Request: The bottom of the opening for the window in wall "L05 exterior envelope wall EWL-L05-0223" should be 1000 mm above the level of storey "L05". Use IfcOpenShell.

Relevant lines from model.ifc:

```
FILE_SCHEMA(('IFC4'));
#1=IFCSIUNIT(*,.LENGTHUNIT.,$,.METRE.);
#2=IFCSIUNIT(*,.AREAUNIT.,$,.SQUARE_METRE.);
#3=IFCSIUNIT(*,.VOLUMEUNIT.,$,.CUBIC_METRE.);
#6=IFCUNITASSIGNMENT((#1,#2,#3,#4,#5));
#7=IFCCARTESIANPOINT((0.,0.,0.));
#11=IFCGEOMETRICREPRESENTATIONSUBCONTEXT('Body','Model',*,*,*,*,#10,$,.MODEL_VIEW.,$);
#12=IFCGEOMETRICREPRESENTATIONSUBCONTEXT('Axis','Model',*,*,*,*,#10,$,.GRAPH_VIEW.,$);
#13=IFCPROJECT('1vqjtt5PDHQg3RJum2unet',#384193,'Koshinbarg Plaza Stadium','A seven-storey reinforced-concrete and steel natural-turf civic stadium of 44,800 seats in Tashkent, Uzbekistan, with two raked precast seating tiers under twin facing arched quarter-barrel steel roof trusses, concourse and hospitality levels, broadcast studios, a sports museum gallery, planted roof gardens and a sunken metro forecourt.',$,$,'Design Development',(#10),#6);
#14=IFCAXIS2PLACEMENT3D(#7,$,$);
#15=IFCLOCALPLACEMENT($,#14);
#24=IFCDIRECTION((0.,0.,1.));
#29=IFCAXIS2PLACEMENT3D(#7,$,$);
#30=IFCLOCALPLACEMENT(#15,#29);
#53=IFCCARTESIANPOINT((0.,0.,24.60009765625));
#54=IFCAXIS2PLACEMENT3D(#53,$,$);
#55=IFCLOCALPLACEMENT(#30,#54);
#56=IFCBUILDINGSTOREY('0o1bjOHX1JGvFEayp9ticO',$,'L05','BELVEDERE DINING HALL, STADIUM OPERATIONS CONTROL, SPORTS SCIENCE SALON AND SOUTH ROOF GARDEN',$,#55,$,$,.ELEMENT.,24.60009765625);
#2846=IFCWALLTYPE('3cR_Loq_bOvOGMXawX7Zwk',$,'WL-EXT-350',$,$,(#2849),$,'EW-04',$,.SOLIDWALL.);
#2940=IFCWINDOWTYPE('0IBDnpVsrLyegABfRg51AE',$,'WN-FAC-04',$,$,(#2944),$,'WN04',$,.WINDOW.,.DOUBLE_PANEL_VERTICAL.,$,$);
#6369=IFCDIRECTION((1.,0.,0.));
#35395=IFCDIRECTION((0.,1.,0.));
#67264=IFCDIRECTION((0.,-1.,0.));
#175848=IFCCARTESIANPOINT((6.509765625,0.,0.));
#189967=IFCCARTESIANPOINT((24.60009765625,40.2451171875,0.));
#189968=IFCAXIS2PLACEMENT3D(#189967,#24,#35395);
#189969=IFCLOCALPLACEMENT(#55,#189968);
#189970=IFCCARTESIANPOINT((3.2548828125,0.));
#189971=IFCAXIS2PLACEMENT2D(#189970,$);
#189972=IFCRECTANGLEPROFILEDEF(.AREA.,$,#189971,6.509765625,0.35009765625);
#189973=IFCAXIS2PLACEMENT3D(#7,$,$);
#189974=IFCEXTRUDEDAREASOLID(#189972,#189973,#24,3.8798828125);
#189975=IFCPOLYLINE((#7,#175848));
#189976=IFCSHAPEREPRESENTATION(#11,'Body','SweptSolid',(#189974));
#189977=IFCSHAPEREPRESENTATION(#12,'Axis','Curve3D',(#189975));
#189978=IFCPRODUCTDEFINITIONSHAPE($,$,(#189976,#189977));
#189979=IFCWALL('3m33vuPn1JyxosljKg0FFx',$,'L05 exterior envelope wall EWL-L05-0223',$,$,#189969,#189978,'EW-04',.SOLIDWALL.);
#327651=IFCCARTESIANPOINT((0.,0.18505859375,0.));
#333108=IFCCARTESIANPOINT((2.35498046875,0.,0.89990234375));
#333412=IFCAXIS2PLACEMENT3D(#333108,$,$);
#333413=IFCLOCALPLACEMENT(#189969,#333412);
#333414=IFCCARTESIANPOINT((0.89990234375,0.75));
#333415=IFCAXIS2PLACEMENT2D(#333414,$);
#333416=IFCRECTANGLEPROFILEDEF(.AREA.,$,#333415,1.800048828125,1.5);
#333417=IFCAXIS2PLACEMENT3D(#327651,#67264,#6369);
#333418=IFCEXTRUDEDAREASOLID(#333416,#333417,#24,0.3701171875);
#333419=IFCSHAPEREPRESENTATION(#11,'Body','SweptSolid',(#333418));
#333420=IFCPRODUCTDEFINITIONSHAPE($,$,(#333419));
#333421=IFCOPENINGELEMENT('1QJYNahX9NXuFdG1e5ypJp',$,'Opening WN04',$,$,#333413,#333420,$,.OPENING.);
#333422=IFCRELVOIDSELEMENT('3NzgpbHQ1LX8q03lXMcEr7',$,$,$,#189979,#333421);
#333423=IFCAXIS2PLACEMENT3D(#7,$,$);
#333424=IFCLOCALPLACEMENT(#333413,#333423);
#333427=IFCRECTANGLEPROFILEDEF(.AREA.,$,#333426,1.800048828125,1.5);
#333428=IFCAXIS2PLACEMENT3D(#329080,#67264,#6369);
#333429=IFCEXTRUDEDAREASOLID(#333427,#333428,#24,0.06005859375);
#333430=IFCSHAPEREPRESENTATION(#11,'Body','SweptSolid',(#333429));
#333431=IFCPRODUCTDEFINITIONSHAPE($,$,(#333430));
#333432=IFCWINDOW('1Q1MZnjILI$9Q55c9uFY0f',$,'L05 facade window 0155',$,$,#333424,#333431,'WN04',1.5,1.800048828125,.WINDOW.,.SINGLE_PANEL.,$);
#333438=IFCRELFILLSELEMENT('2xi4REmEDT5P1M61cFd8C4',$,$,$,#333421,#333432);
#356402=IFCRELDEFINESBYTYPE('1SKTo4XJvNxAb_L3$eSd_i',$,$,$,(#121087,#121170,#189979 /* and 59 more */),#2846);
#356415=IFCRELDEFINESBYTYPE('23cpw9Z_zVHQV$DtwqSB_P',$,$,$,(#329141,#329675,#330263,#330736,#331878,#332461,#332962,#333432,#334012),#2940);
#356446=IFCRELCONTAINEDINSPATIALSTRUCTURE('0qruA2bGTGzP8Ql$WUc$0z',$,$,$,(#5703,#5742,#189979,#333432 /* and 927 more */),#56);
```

```python
import numpy as np
import ifcopenshell
import ifcopenshell.api.geometry
import ifcopenshell.geom
import ifcopenshell.util.element
import ifcopenshell.util.placement
import ifcopenshell.util.shape
import ifcopenshell.util.unit

model = ifcopenshell.open("model.ifc")
unit_scale = ifcopenshell.util.unit.calculate_unit_scale(model)

window = model.by_guid("1Q1MZnjILI$9Q55c9uFY0f")
opening = window.FillsVoids[0].RelatingOpeningElement
storey = ifcopenshell.util.element.get_container(window, ifc_class="IfcBuildingStorey")
level = ifcopenshell.util.placement.get_local_placement(storey.ObjectPlacement)[2, 3]

# The opening's origin need not be at the sill, so measure its lowest point.
shape = ifcopenshell.geom.create_shape(ifcopenshell.geom.settings(), opening)
bottom = ifcopenshell.util.shape.get_shape_bottom_elevation(shape, shape.geometry) / unit_scale
dz = level + 1 / unit_scale - bottom

shift = np.array([0.0, 0.0, dz])
# The window is placed relative to its opening, so it follows when the opening moves.
matrix = ifcopenshell.util.placement.get_local_placement(opening.ObjectPlacement)
matrix[:3, 3] += shift
ifcopenshell.api.geometry.edit_object_placement(
    model, product=opening, matrix=matrix, is_si=False, should_transform_children=True
)

print(f"moved by {dz * unit_scale:+.3f} m")

model.write("model_rev.ifc")
```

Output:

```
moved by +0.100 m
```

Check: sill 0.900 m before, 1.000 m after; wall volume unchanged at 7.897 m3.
